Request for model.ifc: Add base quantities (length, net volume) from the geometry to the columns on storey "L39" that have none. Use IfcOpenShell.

First a look at what the model holds.

```python
import ifcopenshell
import ifcopenshell.util.element
import ifcopenshell.util.unit

model = ifcopenshell.open("model.ifc")
print(model.schema)
for unit_type in ("LENGTHUNIT", "AREAUNIT", "VOLUMEUNIT"):
    print(unit_type, ifcopenshell.util.unit.calculate_unit_scale(model, unit_type))
storey = next(s for s in model.by_type("IfcBuildingStorey") if s.Name == "L39")
columns = [e for e in ifcopenshell.util.element.get_decomposition(storey) if e.is_a("IfcColumn")]
for e in sorted(columns, key=lambda e: e.id()):
    print(e.id(), e.is_a(), e.Name, list(ifcopenshell.util.element.get_psets(e, qtos_only=True)), sep=" | ")
```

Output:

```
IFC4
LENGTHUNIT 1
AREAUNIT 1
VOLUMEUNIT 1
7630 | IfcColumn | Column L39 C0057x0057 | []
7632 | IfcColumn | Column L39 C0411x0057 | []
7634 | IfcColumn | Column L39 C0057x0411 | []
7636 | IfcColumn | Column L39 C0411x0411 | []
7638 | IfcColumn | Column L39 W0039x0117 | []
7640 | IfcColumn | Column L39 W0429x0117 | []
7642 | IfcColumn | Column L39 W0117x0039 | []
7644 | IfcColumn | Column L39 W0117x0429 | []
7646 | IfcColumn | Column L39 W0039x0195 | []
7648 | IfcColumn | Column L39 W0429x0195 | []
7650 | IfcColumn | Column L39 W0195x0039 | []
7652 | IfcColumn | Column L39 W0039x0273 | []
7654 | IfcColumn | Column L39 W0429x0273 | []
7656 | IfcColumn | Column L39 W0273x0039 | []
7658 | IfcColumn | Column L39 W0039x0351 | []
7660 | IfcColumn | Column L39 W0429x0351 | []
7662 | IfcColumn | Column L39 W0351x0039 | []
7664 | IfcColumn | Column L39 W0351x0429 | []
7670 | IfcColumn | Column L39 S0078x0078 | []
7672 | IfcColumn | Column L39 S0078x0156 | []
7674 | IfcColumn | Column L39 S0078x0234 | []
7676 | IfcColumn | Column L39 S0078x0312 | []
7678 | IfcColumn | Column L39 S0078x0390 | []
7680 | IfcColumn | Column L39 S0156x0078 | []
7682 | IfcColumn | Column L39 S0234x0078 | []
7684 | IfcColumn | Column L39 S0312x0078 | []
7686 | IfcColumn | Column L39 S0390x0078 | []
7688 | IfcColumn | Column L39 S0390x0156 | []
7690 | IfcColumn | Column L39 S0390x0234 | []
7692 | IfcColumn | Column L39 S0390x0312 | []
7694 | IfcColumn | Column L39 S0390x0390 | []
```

```python
import ifcopenshell
import ifcopenshell.api.pset
import ifcopenshell.geom
import ifcopenshell.util.element
import ifcopenshell.util.shape
import ifcopenshell.util.unit

model = ifcopenshell.open("model.ifc")
unit_scale = ifcopenshell.util.unit.calculate_unit_scale(model)
volume_scale = ifcopenshell.util.unit.calculate_unit_scale(model, "VOLUMEUNIT")
settings = ifcopenshell.geom.settings()

storey = next(s for s in model.by_type("IfcBuildingStorey") if s.Name == "L39")
columns = [e for e in ifcopenshell.util.element.get_decomposition(storey) if e.is_a("IfcColumn")]

for e in sorted(columns, key=lambda e: e.id()):
    if ifcopenshell.util.element.get_psets(e, qtos_only=True, should_inherit=False):
        continue
    # Geometry comes back in metres, in the element's own axes.
    shape = ifcopenshell.geom.create_shape(settings, e)
    values = {
        "Length": ifcopenshell.util.shape.get_z(shape.geometry) / unit_scale,
        "NetVolume": ifcopenshell.util.shape.get_volume(shape.geometry) / volume_scale,
    }
    qto = ifcopenshell.api.pset.add_qto(model, product=e, name="Qto_ColumnBaseQuantities")
    ifcopenshell.api.pset.edit_qto(model, qto=qto, properties=values)
    print(e.id(), {k: round(v, 3) for k, v in values.items()})

model.write("model_edited.ifc")
```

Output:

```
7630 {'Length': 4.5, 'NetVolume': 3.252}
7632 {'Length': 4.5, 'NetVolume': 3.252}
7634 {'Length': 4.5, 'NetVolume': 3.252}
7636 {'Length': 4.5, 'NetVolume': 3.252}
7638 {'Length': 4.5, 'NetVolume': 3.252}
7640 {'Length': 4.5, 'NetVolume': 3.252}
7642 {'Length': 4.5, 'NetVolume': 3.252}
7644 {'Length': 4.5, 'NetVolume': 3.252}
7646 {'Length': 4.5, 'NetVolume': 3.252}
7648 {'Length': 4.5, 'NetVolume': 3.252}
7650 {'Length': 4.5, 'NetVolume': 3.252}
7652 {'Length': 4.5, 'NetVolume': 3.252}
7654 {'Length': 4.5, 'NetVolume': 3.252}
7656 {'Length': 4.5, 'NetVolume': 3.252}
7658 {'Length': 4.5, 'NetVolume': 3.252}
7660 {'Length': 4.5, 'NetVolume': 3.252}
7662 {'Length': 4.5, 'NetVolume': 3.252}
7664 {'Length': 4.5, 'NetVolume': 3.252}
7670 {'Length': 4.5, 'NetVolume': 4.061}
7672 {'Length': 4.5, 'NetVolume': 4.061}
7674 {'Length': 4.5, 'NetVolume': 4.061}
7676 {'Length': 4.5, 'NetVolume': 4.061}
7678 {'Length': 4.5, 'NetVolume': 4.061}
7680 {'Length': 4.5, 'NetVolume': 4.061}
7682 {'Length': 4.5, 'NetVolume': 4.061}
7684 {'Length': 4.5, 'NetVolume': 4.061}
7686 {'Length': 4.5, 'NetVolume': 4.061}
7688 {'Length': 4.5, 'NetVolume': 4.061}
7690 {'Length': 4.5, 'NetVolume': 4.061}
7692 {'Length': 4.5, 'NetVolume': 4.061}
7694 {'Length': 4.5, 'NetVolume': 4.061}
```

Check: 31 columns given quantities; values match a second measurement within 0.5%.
